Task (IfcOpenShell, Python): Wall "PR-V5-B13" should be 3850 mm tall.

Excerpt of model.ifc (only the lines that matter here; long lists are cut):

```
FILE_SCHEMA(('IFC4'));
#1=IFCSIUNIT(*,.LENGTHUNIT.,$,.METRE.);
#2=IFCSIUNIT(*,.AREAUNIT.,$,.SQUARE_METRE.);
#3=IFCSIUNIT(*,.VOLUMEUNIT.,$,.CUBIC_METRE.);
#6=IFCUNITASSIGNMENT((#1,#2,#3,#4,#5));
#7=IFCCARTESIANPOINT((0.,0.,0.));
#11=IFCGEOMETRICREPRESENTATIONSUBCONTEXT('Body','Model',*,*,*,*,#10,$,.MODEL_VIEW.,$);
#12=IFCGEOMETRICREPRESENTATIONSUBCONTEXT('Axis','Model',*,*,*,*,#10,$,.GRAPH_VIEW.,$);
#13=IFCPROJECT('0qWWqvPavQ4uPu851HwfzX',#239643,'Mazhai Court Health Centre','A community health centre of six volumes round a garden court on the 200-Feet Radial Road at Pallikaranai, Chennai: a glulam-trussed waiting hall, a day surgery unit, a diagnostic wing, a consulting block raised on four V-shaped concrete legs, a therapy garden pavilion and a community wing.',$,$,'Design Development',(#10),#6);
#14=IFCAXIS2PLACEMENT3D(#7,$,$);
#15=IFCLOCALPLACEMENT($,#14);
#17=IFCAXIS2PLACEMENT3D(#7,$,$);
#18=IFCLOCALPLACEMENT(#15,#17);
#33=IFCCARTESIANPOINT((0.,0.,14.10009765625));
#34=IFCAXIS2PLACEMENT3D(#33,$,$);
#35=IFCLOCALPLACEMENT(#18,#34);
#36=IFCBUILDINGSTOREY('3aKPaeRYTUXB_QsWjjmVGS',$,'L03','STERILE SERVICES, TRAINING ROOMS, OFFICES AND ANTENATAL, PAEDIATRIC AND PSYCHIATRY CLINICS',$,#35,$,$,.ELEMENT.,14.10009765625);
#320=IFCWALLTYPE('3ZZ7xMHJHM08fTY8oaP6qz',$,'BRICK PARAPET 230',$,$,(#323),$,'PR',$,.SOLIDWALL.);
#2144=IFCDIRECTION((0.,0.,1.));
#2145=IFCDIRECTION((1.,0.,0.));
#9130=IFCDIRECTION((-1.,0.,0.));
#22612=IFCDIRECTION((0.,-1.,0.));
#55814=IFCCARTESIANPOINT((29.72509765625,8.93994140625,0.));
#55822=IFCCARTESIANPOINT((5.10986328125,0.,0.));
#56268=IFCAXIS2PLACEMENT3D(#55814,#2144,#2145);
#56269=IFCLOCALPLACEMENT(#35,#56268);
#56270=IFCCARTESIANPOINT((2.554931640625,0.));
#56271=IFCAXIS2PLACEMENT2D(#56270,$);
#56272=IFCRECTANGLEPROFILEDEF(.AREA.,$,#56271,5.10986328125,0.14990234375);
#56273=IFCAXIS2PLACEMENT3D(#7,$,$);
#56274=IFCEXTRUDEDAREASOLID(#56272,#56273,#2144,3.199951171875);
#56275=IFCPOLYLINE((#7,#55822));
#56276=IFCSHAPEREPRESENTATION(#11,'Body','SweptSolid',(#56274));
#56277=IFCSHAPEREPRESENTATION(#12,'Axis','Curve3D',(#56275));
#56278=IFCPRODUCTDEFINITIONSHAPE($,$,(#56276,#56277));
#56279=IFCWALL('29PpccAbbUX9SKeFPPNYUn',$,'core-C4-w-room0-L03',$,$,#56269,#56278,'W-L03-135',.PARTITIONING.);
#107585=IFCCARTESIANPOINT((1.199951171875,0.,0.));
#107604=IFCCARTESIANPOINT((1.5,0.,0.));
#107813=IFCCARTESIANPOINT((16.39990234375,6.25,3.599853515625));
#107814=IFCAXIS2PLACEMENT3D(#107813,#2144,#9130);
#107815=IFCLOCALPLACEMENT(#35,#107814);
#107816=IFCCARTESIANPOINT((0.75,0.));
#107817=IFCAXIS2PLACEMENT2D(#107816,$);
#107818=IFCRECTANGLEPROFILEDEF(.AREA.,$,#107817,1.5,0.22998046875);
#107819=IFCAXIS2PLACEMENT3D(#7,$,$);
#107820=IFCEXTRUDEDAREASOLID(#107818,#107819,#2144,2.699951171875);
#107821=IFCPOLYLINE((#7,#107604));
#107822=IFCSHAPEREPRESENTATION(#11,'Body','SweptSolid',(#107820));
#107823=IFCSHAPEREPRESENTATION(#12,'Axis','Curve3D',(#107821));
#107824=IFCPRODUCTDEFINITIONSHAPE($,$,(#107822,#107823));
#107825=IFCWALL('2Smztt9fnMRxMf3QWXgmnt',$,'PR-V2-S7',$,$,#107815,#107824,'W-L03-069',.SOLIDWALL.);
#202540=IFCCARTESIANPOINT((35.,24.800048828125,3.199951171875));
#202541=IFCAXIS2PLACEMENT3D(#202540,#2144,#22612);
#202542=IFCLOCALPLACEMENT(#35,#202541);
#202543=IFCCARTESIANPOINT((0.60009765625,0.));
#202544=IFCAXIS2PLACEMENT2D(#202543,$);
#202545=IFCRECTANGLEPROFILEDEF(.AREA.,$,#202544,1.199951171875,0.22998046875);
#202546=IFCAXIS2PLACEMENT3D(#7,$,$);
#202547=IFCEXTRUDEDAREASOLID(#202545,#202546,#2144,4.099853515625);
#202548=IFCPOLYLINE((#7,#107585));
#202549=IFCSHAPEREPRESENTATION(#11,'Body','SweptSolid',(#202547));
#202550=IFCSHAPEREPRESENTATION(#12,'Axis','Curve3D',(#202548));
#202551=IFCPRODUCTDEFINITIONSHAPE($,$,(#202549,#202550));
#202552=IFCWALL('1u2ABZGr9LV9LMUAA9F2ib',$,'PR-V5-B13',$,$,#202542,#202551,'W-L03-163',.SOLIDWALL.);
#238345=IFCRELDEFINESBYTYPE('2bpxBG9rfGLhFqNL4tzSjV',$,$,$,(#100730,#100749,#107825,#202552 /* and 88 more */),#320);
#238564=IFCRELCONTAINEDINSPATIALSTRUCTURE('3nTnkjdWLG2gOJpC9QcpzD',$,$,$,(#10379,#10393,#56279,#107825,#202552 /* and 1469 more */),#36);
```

```python
import ifcopenshell
import ifcopenshell.geom
import ifcopenshell.util.representation
import ifcopenshell.util.shape
import ifcopenshell.util.unit

model = ifcopenshell.open("model.ifc")
unit_scale = ifcopenshell.util.unit.calculate_unit_scale(model)
settings = ifcopenshell.geom.settings()


def volume(element):
    """Net volume in cubic metres, openings subtracted."""
    shape = ifcopenshell.geom.create_shape(settings, element)
    return ifcopenshell.util.shape.get_volume(shape.geometry)


wall = model.by_guid("1u2ABZGr9LV9LMUAA9F2ib")
before = volume(wall)

body = ifcopenshell.util.representation.get_representation(wall, "Model", "Body")
solid = body.Items[0]
old_height = solid.Depth
solid.Depth = 3.85 / unit_scale
after = volume(wall)

print(f"height {old_height:g} -> {solid.Depth:g}, volume {before:.3f} -> {after:.3f} m3")

model.write("model_v2.ifc")
```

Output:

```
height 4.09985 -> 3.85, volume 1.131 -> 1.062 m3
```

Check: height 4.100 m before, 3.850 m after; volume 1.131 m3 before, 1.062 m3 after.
